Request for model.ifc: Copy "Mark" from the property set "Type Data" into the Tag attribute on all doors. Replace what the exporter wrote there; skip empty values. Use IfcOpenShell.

First a look at what the model holds.

```python
import ifcopenshell
import ifcopenshell.util.element

model = ifcopenshell.open("model.ifc")
print(model.schema)
doors = model.by_type("IfcDoor")
print(len(doors), "doors")
for e in doors[:8]:
    source = ifcopenshell.util.element.get_pset(e, "Type Data", "Mark")
    target = e.Tag
    print(e.id(), repr(source), repr(target), sep=" | ")
```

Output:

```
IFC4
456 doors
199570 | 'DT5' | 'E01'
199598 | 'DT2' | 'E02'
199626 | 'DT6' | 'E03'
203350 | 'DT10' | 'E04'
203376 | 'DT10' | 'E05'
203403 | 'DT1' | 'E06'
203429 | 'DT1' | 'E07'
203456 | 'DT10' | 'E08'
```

```python
import ifcopenshell
import ifcopenshell.util.element

model = ifcopenshell.open("model.ifc")

count = 0
for e in model.by_type("IfcDoor"):
    value = ifcopenshell.util.element.get_pset(e, "Type Data", "Mark")
    current = e.Tag
    if not value or not value.strip() or current == value:
        continue
    e.Tag = value
    count += 1

print(count, "doors updated")

model.write("model-out.ifc")
```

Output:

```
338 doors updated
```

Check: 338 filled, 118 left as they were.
